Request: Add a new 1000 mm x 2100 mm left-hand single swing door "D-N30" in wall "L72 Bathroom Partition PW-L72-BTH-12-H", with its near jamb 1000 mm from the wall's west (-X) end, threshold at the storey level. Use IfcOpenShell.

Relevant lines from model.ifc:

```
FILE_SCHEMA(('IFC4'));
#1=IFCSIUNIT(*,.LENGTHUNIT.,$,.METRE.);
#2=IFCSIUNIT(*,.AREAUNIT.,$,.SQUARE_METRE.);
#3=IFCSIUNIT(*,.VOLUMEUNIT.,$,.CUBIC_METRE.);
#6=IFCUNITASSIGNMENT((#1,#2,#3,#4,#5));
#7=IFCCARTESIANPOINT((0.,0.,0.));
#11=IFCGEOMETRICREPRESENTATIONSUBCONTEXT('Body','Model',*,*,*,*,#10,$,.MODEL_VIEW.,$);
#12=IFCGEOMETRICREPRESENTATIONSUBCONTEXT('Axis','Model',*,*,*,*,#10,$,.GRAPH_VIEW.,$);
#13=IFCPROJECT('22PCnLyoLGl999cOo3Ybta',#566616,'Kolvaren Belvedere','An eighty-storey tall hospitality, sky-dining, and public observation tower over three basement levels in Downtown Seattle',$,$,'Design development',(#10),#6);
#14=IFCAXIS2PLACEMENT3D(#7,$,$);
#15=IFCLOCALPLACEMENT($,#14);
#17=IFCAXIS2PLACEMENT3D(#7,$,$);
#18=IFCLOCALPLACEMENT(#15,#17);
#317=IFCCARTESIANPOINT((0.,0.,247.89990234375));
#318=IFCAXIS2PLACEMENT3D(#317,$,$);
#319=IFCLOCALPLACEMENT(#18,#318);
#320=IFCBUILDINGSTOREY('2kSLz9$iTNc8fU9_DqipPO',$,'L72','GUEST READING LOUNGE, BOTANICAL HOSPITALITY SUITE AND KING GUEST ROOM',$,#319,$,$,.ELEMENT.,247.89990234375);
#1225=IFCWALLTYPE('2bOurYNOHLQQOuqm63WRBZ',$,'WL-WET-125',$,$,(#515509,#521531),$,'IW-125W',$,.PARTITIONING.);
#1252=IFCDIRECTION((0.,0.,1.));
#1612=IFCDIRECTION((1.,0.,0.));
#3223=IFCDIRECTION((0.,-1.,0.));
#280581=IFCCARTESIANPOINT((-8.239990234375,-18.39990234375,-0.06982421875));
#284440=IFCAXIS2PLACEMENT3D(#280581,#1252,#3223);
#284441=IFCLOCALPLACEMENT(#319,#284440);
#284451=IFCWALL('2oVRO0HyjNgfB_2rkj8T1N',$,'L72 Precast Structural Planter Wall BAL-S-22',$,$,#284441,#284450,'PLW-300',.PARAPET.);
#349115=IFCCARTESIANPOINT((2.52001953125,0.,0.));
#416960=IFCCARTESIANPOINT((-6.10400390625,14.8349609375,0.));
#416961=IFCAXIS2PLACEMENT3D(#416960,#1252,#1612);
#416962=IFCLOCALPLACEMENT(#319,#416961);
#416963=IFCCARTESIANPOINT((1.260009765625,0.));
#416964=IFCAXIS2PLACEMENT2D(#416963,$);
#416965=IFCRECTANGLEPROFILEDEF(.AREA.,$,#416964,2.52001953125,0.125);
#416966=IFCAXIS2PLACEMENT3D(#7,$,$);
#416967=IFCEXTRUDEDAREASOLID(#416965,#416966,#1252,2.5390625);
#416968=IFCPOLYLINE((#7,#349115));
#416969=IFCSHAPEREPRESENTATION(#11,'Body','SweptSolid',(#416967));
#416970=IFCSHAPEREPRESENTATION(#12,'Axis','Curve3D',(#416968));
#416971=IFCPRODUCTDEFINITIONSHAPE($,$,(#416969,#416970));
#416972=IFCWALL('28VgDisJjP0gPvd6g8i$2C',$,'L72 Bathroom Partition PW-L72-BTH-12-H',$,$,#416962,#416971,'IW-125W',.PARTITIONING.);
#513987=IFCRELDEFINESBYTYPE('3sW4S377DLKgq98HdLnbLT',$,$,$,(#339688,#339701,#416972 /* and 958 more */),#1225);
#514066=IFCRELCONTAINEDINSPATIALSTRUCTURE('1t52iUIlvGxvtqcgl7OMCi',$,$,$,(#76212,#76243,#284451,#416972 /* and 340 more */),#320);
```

```python
import numpy as np
import ifcopenshell
import ifcopenshell.api.feature
import ifcopenshell.api.geometry
import ifcopenshell.api.root
import ifcopenshell.api.spatial
import ifcopenshell.geom
import ifcopenshell.util.element
import ifcopenshell.util.placement
import ifcopenshell.util.representation
import ifcopenshell.util.shape
import ifcopenshell.util.unit

model = ifcopenshell.open("model.ifc")
unit_scale = ifcopenshell.util.unit.calculate_unit_scale(model)
settings = ifcopenshell.geom.settings()


def volume(element):
    """Net volume in cubic metres, openings subtracted."""
    shape = ifcopenshell.geom.create_shape(settings, element)
    return ifcopenshell.util.shape.get_volume(shape.geometry)


wall = model.by_guid("28VgDisJjP0gPvd6g8i$2C")
storey = ifcopenshell.util.element.get_container(wall, ifc_class="IfcBuildingStorey")
context = ifcopenshell.util.representation.get_context(model, "Model", "Body", "MODEL_VIEW")
before = volume(wall)

width, height, from_end, sill = 1, 2.1, 1, 0.0  # metres

# The wall runs along its own X axis, and the end named is its -X end.
wall_shape = ifcopenshell.geom.create_shape(settings, wall)
x, y, z = ifcopenshell.util.shape.get_vertices(wall_shape.geometry).T
start = x.min() + from_end
face, thickness = float(y.min()), float(y.max() - y.min())
wall_matrix = ifcopenshell.util.placement.get_local_placement(wall.ObjectPlacement)
level = ifcopenshell.util.placement.get_local_placement(storey.ObjectPlacement)[2, 3]


def in_wall(x, y):
    """Placement at x, y metres in the wall's axes, at sill height."""
    matrix = wall_matrix.copy()
    matrix[:, 3] = wall_matrix @ np.array([x / unit_scale, y / unit_scale, 0.0, 1.0])
    matrix[2, 3] = level + sill / unit_scale
    return matrix


# Opening: a box that overshoots both wall faces by 50 mm.
opening = ifcopenshell.api.root.create_entity(model, ifc_class="IfcOpeningElement", predefined_type="OPENING")
box = ifcopenshell.api.geometry.add_wall_representation(
    model, context=context, length=width, height=height, thickness=thickness + 0.1
)
ifcopenshell.api.geometry.assign_representation(model, product=opening, representation=box)
ifcopenshell.api.geometry.edit_object_placement(model, product=opening, matrix=in_wall(start, face - 0.05), is_si=False)
ifcopenshell.api.feature.add_feature(model, feature=opening, element=wall)

door = ifcopenshell.api.root.create_entity(model, ifc_class="IfcDoor", name="D-N30", predefined_type="DOOR")
door.OverallWidth, door.OverallHeight = width / unit_scale, height / unit_scale
door.OperationType = "SINGLE_SWING_LEFT"
body = ifcopenshell.api.geometry.add_door_representation(
    model,
    context=context,
    overall_width=door.OverallWidth,
    overall_height=door.OverallHeight,
    operation_type="SINGLE_SWING_LEFT",
    lining_properties={"LiningDepth": thickness / unit_scale, "ThresholdDepth": thickness / unit_scale},
)
ifcopenshell.api.geometry.assign_representation(model, product=door, representation=body)
ifcopenshell.api.spatial.assign_container(model, products=[door], relating_structure=storey)
ifcopenshell.api.feature.add_filling(model, opening=opening, element=door)

# The lining spans the wall, so the door starts at the wall face.
ifcopenshell.api.geometry.edit_object_placement(model, product=door, matrix=in_wall(start, face), is_si=False)

after = volume(wall)

print(f"wall volume {before:.3f} -> {after:.3f} m3")

model.write("model_edited.ifc")
```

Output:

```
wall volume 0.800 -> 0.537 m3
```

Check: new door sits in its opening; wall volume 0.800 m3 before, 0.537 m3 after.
